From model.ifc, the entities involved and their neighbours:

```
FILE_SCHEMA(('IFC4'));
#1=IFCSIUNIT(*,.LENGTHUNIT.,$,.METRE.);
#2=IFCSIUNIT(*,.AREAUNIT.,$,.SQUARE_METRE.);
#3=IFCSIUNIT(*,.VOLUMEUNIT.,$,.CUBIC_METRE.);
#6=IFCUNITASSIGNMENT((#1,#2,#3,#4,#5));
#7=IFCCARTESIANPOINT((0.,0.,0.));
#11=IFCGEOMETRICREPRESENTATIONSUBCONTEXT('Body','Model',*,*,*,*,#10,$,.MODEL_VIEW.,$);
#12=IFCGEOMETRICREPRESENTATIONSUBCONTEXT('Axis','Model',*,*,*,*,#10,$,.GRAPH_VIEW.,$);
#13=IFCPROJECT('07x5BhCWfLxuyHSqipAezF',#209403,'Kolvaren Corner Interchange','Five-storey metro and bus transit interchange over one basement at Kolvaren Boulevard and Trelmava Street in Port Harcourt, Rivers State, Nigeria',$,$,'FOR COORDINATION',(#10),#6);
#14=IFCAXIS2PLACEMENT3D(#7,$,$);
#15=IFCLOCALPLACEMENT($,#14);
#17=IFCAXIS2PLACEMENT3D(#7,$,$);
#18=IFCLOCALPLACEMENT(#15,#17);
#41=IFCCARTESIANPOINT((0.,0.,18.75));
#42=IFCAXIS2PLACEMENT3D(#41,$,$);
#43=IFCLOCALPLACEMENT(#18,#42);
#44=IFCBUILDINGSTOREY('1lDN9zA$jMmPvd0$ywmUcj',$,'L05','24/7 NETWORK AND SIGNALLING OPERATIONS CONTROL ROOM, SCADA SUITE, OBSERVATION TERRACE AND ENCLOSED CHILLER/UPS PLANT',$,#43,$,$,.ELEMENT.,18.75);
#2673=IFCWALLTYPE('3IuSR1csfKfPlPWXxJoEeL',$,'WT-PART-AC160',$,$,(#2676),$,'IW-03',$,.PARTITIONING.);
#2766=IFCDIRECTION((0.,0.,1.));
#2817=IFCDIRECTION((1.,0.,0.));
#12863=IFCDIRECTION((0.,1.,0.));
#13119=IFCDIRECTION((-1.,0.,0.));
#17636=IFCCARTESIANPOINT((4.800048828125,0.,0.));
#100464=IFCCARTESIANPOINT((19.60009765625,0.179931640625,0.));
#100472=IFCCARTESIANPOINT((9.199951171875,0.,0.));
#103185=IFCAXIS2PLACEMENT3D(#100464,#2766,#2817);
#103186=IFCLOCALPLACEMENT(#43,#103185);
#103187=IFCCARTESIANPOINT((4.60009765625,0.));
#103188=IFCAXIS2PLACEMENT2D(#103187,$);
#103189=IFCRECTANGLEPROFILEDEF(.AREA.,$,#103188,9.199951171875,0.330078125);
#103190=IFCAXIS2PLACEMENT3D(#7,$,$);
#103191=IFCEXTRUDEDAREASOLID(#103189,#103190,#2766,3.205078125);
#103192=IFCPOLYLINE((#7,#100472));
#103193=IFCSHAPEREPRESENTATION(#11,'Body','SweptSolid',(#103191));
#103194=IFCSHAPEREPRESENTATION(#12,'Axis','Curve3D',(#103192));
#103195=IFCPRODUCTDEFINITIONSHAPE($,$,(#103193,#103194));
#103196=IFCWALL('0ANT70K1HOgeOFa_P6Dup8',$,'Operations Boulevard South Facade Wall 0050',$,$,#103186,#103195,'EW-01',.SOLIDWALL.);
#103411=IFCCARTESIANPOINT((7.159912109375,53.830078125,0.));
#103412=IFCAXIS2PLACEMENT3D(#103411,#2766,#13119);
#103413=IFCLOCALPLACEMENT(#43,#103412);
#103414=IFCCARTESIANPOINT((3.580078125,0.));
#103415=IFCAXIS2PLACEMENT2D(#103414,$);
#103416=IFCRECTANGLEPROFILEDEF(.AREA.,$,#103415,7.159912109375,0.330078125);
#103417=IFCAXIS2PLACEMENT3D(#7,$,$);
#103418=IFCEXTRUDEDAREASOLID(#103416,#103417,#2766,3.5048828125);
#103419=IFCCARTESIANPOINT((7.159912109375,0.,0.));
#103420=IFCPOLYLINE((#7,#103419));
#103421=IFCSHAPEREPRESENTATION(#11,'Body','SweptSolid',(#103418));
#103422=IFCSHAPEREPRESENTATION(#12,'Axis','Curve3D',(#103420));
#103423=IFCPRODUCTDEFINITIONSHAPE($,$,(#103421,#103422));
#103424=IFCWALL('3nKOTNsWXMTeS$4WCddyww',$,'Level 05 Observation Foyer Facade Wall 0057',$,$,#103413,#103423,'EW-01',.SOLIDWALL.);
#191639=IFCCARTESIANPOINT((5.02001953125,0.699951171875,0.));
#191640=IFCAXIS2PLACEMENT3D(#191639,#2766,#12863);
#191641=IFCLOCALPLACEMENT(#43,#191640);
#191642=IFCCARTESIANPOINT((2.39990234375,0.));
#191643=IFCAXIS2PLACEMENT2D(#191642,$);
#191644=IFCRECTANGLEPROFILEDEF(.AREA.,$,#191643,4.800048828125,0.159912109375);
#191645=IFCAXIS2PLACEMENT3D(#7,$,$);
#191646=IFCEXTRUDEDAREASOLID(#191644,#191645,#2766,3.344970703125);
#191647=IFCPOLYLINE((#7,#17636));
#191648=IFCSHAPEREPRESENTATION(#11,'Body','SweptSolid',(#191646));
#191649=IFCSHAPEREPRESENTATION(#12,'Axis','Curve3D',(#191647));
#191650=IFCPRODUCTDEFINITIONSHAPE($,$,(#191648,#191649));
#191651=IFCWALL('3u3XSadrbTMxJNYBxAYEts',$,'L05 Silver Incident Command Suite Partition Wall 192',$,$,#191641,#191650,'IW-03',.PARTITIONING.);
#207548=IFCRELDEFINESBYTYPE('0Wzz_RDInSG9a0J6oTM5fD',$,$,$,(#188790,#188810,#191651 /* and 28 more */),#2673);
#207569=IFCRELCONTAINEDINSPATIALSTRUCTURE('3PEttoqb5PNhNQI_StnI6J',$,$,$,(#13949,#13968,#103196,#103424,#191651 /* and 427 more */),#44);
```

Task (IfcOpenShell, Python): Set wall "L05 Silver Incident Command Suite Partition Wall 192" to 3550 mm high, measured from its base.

```python
import ifcopenshell
import ifcopenshell.geom
import ifcopenshell.util.representation
import ifcopenshell.util.shape

model = ifcopenshell.open("model.ifc")
settings = ifcopenshell.geom.settings()


def volume(element):
    """Net volume in cubic metres, openings subtracted."""
    shape = ifcopenshell.geom.create_shape(settings, element)
    return ifcopenshell.util.shape.get_volume(shape.geometry)


wall = model.by_id(191651)
before = volume(wall)

body = ifcopenshell.util.representation.get_representation(wall, "Model", "Body")
solid = body.Items[0]
old_height = solid.Depth
solid.Depth = 3.55
after = volume(wall)

print(f"height {old_height:g} -> {solid.Depth:g}, volume {before:.3f} -> {after:.3f} m3")

model.write("model_updated.ifc")
```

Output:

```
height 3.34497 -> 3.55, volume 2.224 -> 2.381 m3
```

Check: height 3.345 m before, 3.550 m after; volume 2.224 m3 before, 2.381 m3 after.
